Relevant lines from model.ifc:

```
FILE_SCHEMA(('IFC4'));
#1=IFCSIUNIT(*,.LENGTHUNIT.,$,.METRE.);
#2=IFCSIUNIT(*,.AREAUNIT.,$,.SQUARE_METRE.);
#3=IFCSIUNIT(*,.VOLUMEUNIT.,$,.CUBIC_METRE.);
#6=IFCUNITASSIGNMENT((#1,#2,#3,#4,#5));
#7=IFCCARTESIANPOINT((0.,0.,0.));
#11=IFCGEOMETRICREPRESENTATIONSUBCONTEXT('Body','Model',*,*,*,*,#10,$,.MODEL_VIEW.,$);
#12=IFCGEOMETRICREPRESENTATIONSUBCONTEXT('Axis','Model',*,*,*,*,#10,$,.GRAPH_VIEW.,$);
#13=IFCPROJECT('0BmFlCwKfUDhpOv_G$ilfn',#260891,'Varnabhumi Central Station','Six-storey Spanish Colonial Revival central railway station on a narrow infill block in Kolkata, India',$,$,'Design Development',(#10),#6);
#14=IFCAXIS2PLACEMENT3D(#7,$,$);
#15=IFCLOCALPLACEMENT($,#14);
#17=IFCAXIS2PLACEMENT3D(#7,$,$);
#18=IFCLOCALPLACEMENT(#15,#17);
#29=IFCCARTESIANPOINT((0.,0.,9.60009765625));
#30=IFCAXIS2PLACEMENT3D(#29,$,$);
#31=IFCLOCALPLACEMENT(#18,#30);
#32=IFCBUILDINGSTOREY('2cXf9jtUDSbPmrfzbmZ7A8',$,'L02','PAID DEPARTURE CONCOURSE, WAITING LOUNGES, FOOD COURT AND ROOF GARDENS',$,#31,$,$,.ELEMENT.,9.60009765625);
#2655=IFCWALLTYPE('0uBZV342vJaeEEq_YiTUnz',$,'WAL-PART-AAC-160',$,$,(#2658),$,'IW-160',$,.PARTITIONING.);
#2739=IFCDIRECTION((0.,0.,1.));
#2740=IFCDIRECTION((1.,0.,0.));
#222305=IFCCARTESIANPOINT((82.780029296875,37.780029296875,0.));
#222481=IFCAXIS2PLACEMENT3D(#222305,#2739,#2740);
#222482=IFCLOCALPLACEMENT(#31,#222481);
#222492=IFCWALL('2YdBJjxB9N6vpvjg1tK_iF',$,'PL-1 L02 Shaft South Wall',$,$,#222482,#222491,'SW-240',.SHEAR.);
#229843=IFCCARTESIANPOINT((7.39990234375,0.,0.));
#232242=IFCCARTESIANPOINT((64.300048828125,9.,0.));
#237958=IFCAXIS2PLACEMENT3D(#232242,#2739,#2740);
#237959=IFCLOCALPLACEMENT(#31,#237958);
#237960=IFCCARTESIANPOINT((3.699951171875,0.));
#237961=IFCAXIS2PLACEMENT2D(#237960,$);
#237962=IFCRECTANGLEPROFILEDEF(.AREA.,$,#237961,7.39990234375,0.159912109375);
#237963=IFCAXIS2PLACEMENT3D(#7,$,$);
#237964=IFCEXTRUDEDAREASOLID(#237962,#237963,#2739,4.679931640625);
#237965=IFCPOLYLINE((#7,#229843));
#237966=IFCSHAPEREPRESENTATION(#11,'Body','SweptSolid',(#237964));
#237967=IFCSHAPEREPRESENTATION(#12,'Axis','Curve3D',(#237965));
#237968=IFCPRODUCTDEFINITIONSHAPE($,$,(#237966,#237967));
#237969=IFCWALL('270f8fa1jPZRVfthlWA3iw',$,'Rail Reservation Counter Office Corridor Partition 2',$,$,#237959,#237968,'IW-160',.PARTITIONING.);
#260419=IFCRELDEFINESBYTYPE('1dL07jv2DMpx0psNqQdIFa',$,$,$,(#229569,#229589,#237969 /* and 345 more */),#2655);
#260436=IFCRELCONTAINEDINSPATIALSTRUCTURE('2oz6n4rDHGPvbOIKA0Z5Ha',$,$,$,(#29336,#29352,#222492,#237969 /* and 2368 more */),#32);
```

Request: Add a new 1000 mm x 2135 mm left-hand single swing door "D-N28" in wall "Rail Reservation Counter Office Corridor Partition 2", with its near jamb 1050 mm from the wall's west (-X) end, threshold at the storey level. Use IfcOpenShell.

```python
import numpy as np
import ifcopenshell
import ifcopenshell.api.feature
import ifcopenshell.api.geometry
import ifcopenshell.api.root
import ifcopenshell.api.spatial
import ifcopenshell.geom
import ifcopenshell.util.element
import ifcopenshell.util.placement
import ifcopenshell.util.representation
import ifcopenshell.util.shape
import ifcopenshell.util.unit

model = ifcopenshell.open("model.ifc")
unit_scale = ifcopenshell.util.unit.calculate_unit_scale(model)
settings = ifcopenshell.geom.settings()


def volume(element):
    """Net volume in cubic metres, openings subtracted."""
    shape = ifcopenshell.geom.create_shape(settings, element)
    return ifcopenshell.util.shape.get_volume(shape.geometry)


wall = model.by_id(237969)
storey = ifcopenshell.util.element.get_container(wall, ifc_class="IfcBuildingStorey")
context = ifcopenshell.util.representation.get_context(model, "Model", "Body", "MODEL_VIEW")
before = volume(wall)

width, height, from_end, sill = 1, 2.135, 1.05, 0.0  # metres

# The wall runs along its own X axis, and the end named is its -X end.
wall_shape = ifcopenshell.geom.create_shape(settings, wall)
x, y, z = ifcopenshell.util.shape.get_vertices(wall_shape.geometry).T
start = x.min() + from_end
face, thickness = float(y.min()), float(y.max() - y.min())
wall_matrix = ifcopenshell.util.placement.get_local_placement(wall.ObjectPlacement)
level = ifcopenshell.util.placement.get_local_placement(storey.ObjectPlacement)[2, 3]


def in_wall(x, y):
    """Placement at x, y metres in the wall's axes, at sill height."""
    matrix = wall_matrix.copy()
    matrix[:, 3] = wall_matrix @ np.array([x / unit_scale, y / unit_scale, 0.0, 1.0])
    matrix[2, 3] = level + sill / unit_scale
    return matrix


# Opening: a box that overshoots both wall faces by 50 mm.
opening = ifcopenshell.api.root.create_entity(model, ifc_class="IfcOpeningElement", predefined_type="OPENING")
box = ifcopenshell.api.geometry.add_wall_representation(
    model, context=context, length=width, height=height, thickness=thickness + 0.1
)
ifcopenshell.api.geometry.assign_representation(model, product=opening, representation=box)
ifcopenshell.api.geometry.edit_object_placement(model, product=opening, matrix=in_wall(start, face - 0.05), is_si=False)
ifcopenshell.api.feature.add_feature(model, feature=opening, element=wall)

door = ifcopenshell.api.root.create_entity(model, ifc_class="IfcDoor", name="D-N28", predefined_type="DOOR")
door.OverallWidth, door.OverallHeight = width / unit_scale, height / unit_scale
door.OperationType = "SINGLE_SWING_LEFT"
body = ifcopenshell.api.geometry.add_door_representation(
    model,
    context=context,
    overall_width=door.OverallWidth,
    overall_height=door.OverallHeight,
    operation_type="SINGLE_SWING_LEFT",
    lining_properties={"LiningDepth": thickness / unit_scale, "ThresholdDepth": thickness / unit_scale},
)
ifcopenshell.api.geometry.assign_representation(model, product=door, representation=body)
ifcopenshell.api.spatial.assign_container(model, products=[door], relating_structure=storey)
ifcopenshell.api.feature.add_filling(model, opening=opening, element=door)

# The lining spans the wall, so the door starts at the wall face.
ifcopenshell.api.geometry.edit_object_placement(model, product=door, matrix=in_wall(start, face), is_si=False)

after = volume(wall)

print(f"wall volume {before:.3f} -> {after:.3f} m3")

model.write("model_v2.ifc")
```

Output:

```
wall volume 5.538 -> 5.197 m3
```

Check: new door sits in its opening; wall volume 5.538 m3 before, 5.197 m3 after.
